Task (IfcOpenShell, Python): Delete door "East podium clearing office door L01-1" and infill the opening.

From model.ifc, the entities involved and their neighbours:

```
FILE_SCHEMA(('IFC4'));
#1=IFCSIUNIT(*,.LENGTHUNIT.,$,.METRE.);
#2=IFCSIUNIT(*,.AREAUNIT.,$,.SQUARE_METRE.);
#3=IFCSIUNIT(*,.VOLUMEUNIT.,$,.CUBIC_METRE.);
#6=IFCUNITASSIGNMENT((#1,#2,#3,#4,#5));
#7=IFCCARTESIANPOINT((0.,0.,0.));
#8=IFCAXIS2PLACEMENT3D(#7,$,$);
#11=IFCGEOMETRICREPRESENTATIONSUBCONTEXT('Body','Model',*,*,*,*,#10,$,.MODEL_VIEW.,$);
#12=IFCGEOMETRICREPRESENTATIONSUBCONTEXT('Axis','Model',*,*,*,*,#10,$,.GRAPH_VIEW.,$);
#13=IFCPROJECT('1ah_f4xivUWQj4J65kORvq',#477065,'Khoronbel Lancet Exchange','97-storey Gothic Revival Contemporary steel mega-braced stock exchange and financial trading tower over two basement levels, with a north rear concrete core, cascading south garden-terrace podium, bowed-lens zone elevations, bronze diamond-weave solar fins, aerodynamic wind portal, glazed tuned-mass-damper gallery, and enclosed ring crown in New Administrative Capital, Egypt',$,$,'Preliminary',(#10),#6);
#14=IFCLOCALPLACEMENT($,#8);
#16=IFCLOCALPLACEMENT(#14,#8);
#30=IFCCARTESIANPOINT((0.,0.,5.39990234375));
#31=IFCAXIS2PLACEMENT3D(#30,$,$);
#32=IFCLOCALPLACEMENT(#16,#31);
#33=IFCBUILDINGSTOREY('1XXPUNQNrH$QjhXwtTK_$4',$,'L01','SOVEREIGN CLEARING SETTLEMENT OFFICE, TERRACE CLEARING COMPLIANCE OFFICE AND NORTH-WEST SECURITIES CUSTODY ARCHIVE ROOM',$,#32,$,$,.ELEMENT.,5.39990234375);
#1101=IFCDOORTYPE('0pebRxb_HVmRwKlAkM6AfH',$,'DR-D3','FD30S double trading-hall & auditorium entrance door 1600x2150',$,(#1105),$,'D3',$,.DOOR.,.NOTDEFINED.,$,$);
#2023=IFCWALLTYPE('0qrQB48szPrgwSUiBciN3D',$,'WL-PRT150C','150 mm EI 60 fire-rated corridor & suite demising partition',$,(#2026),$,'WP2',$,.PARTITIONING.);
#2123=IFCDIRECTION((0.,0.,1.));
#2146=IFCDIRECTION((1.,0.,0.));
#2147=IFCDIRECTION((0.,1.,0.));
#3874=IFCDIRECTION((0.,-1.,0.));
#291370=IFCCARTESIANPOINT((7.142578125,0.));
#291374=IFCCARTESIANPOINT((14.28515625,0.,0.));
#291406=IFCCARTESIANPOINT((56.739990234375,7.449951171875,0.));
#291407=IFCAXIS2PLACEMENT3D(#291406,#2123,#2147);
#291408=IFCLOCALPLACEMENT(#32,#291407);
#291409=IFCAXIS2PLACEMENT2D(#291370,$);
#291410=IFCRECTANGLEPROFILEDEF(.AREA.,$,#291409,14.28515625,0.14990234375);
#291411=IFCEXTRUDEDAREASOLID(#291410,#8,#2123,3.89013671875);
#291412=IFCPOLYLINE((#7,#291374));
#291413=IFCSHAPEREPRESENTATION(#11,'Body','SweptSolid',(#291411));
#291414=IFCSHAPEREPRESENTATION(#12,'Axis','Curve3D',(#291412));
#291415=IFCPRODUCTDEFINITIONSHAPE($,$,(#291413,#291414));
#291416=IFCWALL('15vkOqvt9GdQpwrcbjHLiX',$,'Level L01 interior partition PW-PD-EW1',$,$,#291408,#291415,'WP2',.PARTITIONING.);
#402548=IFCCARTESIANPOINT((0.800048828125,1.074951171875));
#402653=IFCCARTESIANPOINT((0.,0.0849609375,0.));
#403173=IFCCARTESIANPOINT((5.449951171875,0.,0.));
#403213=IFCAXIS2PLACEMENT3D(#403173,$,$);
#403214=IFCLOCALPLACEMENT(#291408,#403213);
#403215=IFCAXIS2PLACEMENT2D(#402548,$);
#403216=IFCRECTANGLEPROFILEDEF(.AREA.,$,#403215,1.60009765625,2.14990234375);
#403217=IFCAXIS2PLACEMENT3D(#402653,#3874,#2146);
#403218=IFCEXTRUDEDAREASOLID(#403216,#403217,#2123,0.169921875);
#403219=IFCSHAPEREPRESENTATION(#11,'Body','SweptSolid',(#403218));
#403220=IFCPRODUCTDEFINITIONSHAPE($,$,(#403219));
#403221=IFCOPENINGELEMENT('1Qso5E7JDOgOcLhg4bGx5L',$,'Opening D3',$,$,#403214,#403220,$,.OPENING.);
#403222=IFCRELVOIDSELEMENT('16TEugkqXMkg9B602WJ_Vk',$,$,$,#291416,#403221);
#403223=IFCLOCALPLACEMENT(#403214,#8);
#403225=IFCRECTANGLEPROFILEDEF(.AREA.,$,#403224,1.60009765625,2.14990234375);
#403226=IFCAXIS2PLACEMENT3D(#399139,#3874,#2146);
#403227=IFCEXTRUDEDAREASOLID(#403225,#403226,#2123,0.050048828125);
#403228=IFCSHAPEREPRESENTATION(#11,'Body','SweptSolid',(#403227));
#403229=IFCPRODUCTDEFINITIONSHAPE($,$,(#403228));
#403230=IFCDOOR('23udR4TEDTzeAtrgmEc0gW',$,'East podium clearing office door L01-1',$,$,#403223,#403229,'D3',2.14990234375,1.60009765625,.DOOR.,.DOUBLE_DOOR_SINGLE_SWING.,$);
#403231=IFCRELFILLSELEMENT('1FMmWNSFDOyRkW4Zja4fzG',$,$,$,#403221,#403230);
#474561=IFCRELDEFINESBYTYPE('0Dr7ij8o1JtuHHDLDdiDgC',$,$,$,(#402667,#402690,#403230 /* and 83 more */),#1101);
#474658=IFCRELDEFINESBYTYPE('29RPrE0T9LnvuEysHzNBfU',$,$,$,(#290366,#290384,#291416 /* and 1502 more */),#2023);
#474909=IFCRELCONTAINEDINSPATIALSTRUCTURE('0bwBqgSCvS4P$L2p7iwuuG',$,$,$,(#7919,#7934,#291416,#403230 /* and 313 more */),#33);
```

```python
import ifcopenshell
import ifcopenshell.api.feature
import ifcopenshell.api.root
import ifcopenshell.geom
import ifcopenshell.util.shape

model = ifcopenshell.open("model.ifc")
settings = ifcopenshell.geom.settings()


def volume(element):
    """Net volume in cubic metres, openings subtracted."""
    shape = ifcopenshell.geom.create_shape(settings, element)
    return ifcopenshell.util.shape.get_volume(shape.geometry)


door = model.by_guid("23udR4TEDTzeAtrgmEc0gW")
opening = door.FillsVoids[0].RelatingOpeningElement
wall = opening.VoidsElements[0].RelatingBuildingElement
before = volume(wall)

ifcopenshell.api.root.remove_product(model, product=door)
ifcopenshell.api.feature.remove_feature(model, feature=opening)

after = volume(wall)

print(f"wall volume {before:.3f} -> {after:.3f} m3")

model.write("model_edited.ifc")
```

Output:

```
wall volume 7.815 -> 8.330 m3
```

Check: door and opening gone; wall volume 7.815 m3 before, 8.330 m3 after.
